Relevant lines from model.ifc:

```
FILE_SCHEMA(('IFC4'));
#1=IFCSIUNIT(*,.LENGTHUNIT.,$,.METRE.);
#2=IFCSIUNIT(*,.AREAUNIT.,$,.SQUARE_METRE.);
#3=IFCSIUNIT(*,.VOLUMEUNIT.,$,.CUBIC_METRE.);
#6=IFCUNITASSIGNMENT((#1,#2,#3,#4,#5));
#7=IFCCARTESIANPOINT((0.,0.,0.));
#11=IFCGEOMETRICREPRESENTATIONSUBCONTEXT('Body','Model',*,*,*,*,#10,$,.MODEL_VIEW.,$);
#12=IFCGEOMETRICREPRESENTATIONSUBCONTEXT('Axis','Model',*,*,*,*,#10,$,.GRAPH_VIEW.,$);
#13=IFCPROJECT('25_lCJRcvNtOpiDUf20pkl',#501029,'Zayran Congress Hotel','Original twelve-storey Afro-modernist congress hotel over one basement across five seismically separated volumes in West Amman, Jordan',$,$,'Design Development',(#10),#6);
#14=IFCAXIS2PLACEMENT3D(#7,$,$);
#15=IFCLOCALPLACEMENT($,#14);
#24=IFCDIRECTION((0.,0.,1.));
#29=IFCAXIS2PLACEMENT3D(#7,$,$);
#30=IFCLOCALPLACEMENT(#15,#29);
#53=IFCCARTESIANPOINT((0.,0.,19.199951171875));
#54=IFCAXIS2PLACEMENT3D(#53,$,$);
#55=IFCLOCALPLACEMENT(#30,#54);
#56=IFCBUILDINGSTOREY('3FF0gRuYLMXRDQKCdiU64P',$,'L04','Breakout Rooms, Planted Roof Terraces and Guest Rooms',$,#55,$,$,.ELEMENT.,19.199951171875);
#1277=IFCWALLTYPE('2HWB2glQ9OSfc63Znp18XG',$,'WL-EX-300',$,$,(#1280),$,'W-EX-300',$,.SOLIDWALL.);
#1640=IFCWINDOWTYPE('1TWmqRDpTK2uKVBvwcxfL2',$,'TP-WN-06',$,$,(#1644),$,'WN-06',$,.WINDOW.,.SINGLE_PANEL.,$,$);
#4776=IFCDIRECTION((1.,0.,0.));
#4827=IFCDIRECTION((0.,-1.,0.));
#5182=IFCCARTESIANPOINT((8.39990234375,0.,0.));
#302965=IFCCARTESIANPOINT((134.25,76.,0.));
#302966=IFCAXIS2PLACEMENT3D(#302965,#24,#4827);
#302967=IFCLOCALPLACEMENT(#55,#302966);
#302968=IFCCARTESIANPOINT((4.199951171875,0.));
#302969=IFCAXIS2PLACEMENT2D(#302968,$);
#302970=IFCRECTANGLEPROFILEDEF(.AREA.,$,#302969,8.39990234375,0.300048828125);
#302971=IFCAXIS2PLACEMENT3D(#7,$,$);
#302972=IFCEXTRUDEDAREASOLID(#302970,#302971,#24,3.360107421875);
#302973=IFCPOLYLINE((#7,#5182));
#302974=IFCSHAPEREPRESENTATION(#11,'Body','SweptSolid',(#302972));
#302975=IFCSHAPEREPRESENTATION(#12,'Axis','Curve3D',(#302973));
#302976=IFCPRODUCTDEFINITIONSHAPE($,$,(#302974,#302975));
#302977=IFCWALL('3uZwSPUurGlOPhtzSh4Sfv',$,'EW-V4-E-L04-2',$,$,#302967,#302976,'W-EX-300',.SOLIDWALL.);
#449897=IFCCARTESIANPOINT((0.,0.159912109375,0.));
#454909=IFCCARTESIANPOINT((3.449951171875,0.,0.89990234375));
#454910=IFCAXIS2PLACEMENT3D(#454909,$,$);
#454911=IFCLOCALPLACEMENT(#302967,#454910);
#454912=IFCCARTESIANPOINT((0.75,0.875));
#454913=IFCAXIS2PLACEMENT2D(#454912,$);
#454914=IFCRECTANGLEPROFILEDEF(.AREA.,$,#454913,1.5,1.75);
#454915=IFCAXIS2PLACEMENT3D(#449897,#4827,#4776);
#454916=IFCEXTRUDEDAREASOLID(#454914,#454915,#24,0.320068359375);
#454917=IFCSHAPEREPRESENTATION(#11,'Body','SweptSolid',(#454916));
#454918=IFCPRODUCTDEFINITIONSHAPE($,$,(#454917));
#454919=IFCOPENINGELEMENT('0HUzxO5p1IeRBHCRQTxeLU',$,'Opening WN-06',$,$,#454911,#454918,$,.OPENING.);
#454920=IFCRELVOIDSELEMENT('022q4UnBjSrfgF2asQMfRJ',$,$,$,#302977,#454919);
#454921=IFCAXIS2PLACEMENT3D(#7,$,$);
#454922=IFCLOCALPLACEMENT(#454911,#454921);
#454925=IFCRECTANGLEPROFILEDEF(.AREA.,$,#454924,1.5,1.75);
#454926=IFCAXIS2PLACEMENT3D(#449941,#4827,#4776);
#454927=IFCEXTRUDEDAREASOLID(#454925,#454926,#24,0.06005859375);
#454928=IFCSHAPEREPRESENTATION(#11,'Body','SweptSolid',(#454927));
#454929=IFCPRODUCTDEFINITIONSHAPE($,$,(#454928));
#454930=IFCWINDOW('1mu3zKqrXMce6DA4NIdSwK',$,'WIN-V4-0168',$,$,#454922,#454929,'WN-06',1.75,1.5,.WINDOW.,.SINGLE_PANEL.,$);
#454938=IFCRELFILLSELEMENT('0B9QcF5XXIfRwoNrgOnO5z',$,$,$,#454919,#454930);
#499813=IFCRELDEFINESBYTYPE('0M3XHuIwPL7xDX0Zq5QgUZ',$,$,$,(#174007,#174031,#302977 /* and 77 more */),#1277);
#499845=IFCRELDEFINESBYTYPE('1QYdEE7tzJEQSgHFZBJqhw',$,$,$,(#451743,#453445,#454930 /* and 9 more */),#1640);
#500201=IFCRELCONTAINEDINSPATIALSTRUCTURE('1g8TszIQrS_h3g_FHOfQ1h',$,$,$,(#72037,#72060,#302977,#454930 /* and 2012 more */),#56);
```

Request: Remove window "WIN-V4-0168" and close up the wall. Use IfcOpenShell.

```python
import ifcopenshell
import ifcopenshell.api.feature
import ifcopenshell.api.root
import ifcopenshell.geom
import ifcopenshell.util.shape

model = ifcopenshell.open("model.ifc")
settings = ifcopenshell.geom.settings()


def volume(element):
    """Net volume in cubic metres, openings subtracted."""
    shape = ifcopenshell.geom.create_shape(settings, element)
    return ifcopenshell.util.shape.get_volume(shape.geometry)


window = model.by_guid("1mu3zKqrXMce6DA4NIdSwK")
opening = window.FillsVoids[0].RelatingOpeningElement
wall = opening.VoidsElements[0].RelatingBuildingElement
before = volume(wall)

ifcopenshell.api.root.remove_product(model, product=window)
ifcopenshell.api.feature.remove_feature(model, feature=opening)

after = volume(wall)

print(f"wall volume {before:.3f} -> {after:.3f} m3")

model.write("model-out.ifc")
```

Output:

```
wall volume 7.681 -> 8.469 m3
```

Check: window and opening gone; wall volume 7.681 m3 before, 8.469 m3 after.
